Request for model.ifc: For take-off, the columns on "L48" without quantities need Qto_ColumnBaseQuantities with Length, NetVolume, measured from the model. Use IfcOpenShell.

First a look at what the model holds.

```python
import ifcopenshell
import ifcopenshell.util.element
import ifcopenshell.util.unit

model = ifcopenshell.open("model.ifc")
print(model.schema)
for unit_type in ("LENGTHUNIT", "AREAUNIT", "VOLUMEUNIT"):
    print(unit_type, ifcopenshell.util.unit.calculate_unit_scale(model, unit_type))
storey = next(s for s in model.by_type("IfcBuildingStorey") if s.Name == "L48")
columns = [e for e in ifcopenshell.util.element.get_decomposition(storey) if e.is_a("IfcColumn")]
for e in sorted(columns, key=lambda e: e.id()):
    print(e.id(), e.is_a(), e.Name, list(ifcopenshell.util.element.get_psets(e, qtos_only=True)), sep=" | ")
```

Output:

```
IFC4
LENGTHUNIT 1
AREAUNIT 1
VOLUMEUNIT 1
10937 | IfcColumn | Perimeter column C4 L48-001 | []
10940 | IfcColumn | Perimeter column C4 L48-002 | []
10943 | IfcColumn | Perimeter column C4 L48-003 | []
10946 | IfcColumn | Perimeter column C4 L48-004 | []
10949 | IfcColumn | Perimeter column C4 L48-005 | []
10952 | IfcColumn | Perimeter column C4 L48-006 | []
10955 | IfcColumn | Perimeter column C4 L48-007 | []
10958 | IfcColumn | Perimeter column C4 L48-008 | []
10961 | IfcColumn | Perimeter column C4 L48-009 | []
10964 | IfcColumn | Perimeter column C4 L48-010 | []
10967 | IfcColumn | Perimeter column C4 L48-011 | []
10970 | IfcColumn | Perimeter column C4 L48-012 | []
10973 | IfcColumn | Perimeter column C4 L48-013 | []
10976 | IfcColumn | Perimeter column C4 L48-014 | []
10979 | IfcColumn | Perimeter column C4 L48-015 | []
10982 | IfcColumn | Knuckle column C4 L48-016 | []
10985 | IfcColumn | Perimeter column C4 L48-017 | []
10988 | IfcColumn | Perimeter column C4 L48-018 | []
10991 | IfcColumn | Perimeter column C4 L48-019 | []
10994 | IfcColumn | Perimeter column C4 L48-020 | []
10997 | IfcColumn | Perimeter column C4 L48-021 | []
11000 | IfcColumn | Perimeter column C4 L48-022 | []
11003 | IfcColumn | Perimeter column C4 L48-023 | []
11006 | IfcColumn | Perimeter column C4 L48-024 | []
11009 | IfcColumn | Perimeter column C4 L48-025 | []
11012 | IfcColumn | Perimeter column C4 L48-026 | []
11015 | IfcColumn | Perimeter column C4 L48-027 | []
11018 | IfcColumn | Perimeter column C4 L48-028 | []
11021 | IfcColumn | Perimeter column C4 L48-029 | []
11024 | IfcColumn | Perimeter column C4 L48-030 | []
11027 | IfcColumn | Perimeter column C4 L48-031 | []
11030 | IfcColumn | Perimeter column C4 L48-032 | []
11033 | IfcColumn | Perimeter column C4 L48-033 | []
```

```python
import ifcopenshell
import ifcopenshell.api.pset
import ifcopenshell.geom
import ifcopenshell.util.element
import ifcopenshell.util.shape
import ifcopenshell.util.unit

model = ifcopenshell.open("model.ifc")
unit_scale = ifcopenshell.util.unit.calculate_unit_scale(model)
volume_scale = ifcopenshell.util.unit.calculate_unit_scale(model, "VOLUMEUNIT")
settings = ifcopenshell.geom.settings()

storey = next(s for s in model.by_type("IfcBuildingStorey") if s.Name == "L48")
columns = [e for e in ifcopenshell.util.element.get_decomposition(storey) if e.is_a("IfcColumn")]

for e in sorted(columns, key=lambda e: e.id()):
    if ifcopenshell.util.element.get_psets(e, qtos_only=True, should_inherit=False):
        continue
    # Geometry comes back in metres, in the element's own axes.
    shape = ifcopenshell.geom.create_shape(settings, e)
    values = {
        "Length": ifcopenshell.util.shape.get_z(shape.geometry) / unit_scale,
        "NetVolume": ifcopenshell.util.shape.get_volume(shape.geometry) / volume_scale,
    }
    qto = ifcopenshell.api.pset.add_qto(model, product=e, name="Qto_ColumnBaseQuantities")
    ifcopenshell.api.pset.edit_qto(model, qto=qto, properties=values)
    print(e.id(), {k: round(v, 3) for k, v in values.items()})

model.write("model-out.ifc")
```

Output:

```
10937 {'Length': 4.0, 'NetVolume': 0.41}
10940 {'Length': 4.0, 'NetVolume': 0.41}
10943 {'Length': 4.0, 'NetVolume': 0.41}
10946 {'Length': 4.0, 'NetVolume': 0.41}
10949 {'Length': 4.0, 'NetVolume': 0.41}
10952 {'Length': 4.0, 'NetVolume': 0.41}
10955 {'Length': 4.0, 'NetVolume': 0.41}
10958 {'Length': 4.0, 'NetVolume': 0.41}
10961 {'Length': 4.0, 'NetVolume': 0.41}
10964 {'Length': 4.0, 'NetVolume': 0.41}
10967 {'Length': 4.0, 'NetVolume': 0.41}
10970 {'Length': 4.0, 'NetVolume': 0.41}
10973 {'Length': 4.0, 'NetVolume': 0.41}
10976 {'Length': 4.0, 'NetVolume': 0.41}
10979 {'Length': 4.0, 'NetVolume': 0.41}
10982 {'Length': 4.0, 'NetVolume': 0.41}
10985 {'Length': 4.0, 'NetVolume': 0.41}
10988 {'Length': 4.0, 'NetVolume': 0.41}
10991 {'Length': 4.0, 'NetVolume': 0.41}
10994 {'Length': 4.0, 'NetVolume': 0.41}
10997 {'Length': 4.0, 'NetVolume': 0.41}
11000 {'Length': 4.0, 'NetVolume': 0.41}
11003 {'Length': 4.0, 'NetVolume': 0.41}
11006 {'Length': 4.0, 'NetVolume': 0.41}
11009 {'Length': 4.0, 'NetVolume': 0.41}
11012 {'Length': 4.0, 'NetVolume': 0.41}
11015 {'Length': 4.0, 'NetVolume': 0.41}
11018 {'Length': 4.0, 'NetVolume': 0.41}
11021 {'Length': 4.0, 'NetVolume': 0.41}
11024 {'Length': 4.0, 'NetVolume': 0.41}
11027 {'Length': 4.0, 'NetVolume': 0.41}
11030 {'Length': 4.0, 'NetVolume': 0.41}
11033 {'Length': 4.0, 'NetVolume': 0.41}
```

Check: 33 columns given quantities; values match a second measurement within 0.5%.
